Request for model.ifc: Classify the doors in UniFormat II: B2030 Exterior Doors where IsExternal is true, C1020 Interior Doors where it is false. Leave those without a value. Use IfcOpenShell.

First a look at what the model holds.

```python
import ifcopenshell
import ifcopenshell.util.element

model = ifcopenshell.open("model.ifc")
print(model.schema)
print("classifications:", [c.Name for c in model.by_type("IfcClassification")])
values = [ifcopenshell.util.element.get_pset(e, "Pset_DoorCommon", "IsExternal") for e in model.by_type("IfcDoor")]
for value in (True, False, None):
    print("IsExternal", value, values.count(value))
```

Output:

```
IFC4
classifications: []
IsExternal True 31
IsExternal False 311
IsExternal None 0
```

```python
import ifcopenshell
import ifcopenshell.api.classification
import ifcopenshell.util.element

model = ifcopenshell.open("model.ifc")

system = ifcopenshell.api.classification.add_classification(model, classification="UniFormat II")

doors = model.by_type("IfcDoor")
external = {e: ifcopenshell.util.element.get_pset(e, "Pset_DoorCommon", "IsExternal") for e in doors}
for flag, code, name in ((True, "B2030", "Exterior Doors"), (False, "C1020", "Interior Doors")):
    products = [e for e in doors if external[e] is flag]
    ifcopenshell.api.classification.add_reference(
        model, products=products, classification=system, identification=code, name=name
    )
    print(code, len(products))

model.write("model-out.ifc")
```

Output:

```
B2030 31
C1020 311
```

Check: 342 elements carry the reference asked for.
